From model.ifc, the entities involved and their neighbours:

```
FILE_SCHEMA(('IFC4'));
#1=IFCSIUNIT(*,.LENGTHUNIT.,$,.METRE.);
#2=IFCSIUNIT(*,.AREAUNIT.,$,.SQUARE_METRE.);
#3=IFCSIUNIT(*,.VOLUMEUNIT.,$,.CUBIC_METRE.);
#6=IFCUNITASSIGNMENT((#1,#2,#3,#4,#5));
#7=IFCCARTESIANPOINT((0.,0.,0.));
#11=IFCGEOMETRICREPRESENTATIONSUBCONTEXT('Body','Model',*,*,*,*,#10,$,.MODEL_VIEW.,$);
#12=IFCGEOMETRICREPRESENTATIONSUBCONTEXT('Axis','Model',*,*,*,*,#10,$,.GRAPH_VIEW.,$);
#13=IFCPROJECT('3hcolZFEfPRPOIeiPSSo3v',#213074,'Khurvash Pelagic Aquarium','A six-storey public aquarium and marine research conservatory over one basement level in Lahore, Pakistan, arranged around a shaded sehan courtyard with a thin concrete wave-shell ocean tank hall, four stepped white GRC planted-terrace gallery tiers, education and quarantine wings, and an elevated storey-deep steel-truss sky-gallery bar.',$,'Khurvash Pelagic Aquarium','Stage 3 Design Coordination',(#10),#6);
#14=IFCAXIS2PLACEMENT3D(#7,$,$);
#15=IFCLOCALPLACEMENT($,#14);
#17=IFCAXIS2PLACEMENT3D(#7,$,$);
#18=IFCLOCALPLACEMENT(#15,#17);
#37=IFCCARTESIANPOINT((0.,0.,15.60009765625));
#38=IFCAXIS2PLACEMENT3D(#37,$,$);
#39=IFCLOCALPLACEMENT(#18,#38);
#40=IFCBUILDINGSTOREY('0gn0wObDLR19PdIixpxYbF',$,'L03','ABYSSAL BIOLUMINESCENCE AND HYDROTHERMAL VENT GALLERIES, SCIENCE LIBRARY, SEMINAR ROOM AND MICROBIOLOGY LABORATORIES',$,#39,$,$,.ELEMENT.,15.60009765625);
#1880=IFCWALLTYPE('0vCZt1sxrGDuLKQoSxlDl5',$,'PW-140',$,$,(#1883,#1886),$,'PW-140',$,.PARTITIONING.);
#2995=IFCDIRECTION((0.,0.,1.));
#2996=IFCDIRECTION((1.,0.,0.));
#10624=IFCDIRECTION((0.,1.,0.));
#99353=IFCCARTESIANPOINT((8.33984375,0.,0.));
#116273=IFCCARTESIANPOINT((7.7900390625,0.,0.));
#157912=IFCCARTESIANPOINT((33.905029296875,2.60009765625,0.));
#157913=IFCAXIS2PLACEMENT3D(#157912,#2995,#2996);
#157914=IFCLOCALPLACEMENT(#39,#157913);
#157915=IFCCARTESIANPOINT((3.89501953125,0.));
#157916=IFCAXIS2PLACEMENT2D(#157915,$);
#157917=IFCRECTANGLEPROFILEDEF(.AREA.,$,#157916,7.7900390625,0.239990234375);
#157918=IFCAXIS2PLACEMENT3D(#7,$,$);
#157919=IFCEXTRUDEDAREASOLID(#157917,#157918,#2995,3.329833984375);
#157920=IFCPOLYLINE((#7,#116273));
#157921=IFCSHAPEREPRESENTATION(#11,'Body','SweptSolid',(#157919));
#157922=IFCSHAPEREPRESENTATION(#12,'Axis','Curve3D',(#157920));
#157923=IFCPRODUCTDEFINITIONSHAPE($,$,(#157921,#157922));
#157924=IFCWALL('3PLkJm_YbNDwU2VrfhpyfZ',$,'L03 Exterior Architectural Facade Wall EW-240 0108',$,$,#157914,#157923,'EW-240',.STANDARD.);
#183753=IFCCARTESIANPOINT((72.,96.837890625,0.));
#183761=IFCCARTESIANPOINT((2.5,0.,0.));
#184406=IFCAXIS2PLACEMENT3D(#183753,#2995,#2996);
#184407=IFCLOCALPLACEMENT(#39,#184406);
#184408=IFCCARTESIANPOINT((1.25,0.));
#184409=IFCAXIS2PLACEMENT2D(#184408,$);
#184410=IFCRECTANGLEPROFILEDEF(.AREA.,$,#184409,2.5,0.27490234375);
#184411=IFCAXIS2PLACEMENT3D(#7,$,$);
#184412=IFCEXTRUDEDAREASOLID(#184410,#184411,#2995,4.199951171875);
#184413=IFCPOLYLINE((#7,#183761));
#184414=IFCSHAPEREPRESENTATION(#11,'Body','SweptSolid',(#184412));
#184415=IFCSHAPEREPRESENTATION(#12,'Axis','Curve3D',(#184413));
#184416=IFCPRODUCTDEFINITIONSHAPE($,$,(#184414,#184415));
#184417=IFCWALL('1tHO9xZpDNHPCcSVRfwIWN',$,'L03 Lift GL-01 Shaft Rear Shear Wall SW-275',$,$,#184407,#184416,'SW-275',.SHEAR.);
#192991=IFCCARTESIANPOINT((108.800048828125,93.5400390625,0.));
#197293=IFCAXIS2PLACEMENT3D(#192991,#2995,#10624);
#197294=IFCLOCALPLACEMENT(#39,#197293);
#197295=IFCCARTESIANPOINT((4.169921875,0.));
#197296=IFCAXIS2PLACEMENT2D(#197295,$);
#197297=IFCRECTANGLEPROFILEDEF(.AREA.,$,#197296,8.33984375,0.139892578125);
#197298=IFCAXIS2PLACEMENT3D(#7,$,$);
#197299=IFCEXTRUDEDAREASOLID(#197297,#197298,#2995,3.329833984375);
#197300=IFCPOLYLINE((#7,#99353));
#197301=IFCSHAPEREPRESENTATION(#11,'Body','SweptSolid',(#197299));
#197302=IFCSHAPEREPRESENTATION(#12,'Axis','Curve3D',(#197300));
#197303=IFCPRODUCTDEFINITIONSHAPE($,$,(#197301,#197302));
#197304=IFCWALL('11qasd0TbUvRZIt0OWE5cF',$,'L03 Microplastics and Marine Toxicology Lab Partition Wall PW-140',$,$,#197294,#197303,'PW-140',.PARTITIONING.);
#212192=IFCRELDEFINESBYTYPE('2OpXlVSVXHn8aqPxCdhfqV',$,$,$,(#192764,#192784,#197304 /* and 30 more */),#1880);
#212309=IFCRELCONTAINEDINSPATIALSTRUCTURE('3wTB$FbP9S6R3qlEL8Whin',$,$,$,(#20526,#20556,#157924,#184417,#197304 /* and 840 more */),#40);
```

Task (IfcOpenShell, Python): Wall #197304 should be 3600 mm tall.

```python
import ifcopenshell
import ifcopenshell.geom
import ifcopenshell.util.representation
import ifcopenshell.util.shape
import ifcopenshell.util.unit

model = ifcopenshell.open("model.ifc")
unit_scale = ifcopenshell.util.unit.calculate_unit_scale(model)
settings = ifcopenshell.geom.settings()


def volume(element):
    """Net volume in cubic metres, openings subtracted."""
    shape = ifcopenshell.geom.create_shape(settings, element)
    return ifcopenshell.util.shape.get_volume(shape.geometry)


wall = model.by_guid("11qasd0TbUvRZIt0OWE5cF")
before = volume(wall)

body = ifcopenshell.util.representation.get_representation(wall, "Model", "Body")
solid = body.Items[0]
old_height = solid.Depth
solid.Depth = 3.6 / unit_scale
after = volume(wall)

print(f"height {old_height:g} -> {solid.Depth:g}, volume {before:.3f} -> {after:.3f} m3")

model.write("model-out.ifc")
```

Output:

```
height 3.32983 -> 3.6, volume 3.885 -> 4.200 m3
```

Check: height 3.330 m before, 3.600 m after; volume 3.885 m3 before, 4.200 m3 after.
